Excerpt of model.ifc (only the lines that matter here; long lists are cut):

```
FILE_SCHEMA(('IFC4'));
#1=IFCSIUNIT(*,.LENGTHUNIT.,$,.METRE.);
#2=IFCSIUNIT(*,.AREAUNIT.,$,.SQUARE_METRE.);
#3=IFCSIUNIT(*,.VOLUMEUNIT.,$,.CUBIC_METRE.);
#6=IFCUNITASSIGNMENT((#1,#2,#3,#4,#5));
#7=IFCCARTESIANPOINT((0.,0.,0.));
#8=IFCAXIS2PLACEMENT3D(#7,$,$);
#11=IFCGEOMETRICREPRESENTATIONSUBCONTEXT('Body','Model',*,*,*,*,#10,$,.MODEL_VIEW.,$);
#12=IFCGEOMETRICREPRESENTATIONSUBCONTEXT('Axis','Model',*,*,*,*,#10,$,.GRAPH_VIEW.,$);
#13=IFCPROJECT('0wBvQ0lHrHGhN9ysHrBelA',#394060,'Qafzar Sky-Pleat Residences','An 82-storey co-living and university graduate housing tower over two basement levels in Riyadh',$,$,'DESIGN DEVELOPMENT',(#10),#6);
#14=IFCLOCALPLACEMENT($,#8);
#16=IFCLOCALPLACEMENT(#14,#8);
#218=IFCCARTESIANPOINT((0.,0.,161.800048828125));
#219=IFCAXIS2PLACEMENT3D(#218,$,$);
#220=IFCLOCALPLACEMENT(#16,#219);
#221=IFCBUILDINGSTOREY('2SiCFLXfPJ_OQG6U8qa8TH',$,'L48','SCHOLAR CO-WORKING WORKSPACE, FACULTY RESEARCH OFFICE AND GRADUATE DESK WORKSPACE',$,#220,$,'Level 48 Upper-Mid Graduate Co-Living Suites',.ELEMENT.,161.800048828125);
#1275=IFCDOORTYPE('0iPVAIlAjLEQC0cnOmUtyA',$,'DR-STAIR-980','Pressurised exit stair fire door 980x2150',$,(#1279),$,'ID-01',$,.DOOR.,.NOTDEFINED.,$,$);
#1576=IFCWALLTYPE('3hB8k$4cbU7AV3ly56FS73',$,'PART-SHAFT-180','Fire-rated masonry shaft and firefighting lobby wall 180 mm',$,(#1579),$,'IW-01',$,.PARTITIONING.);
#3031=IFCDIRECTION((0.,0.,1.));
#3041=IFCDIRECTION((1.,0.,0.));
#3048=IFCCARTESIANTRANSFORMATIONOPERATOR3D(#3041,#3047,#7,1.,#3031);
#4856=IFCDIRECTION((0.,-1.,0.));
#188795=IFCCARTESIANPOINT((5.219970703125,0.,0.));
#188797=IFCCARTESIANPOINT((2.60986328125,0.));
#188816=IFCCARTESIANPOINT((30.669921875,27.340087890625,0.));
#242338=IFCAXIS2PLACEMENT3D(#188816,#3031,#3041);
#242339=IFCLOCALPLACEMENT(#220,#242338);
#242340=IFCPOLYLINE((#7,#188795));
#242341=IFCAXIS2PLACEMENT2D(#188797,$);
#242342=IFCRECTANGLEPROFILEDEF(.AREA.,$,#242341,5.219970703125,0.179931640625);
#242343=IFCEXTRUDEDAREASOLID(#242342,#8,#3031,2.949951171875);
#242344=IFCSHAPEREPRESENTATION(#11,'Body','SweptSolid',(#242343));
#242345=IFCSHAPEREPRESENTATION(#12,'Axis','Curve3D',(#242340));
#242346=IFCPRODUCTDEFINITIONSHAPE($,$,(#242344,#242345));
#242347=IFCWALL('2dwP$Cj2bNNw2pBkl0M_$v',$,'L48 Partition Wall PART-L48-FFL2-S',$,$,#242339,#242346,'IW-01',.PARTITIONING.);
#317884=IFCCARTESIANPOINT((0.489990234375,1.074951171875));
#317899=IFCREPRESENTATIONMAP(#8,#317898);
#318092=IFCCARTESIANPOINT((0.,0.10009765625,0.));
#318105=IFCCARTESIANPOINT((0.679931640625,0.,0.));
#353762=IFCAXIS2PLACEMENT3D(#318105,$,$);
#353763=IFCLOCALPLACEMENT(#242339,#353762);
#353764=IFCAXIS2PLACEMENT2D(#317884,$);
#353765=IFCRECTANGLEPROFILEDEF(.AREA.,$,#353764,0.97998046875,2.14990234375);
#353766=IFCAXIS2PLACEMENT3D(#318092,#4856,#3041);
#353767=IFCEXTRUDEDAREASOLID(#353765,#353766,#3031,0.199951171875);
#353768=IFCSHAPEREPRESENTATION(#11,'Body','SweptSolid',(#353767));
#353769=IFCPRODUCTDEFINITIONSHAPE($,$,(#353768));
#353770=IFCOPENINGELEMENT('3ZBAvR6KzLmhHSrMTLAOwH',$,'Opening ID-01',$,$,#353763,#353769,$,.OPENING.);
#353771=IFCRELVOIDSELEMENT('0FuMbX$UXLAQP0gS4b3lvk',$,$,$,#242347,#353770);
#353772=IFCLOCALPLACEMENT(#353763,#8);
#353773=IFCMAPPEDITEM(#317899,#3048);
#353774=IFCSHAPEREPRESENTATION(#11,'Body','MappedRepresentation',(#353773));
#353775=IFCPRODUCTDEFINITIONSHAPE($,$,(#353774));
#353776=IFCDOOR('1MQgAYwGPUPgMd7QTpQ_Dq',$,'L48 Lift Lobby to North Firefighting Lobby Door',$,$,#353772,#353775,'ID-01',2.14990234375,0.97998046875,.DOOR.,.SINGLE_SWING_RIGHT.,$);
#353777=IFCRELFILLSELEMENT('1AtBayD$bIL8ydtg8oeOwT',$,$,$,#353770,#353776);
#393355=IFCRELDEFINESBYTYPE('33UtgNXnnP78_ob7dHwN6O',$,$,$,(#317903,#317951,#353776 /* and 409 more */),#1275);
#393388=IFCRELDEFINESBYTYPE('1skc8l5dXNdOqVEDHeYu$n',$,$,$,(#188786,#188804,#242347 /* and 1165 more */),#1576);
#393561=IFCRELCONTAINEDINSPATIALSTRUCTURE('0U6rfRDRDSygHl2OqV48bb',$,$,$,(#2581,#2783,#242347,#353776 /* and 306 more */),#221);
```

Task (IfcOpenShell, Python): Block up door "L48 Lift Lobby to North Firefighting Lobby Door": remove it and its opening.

```python
import ifcopenshell
import ifcopenshell.api.feature
import ifcopenshell.api.root
import ifcopenshell.geom
import ifcopenshell.util.shape

model = ifcopenshell.open("model.ifc")
settings = ifcopenshell.geom.settings()


def volume(element):
    """Net volume in cubic metres, openings subtracted."""
    shape = ifcopenshell.geom.create_shape(settings, element)
    return ifcopenshell.util.shape.get_volume(shape.geometry)


door = model.by_id(353776)
opening = door.FillsVoids[0].RelatingOpeningElement
wall = opening.VoidsElements[0].RelatingBuildingElement
before = volume(wall)

ifcopenshell.api.root.remove_product(model, product=door)
ifcopenshell.api.feature.remove_feature(model, feature=opening)

after = volume(wall)

print(f"wall volume {before:.3f} -> {after:.3f} m3")

model.write("model_v2.ifc")
```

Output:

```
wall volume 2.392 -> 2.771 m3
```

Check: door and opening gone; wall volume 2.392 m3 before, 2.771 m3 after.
